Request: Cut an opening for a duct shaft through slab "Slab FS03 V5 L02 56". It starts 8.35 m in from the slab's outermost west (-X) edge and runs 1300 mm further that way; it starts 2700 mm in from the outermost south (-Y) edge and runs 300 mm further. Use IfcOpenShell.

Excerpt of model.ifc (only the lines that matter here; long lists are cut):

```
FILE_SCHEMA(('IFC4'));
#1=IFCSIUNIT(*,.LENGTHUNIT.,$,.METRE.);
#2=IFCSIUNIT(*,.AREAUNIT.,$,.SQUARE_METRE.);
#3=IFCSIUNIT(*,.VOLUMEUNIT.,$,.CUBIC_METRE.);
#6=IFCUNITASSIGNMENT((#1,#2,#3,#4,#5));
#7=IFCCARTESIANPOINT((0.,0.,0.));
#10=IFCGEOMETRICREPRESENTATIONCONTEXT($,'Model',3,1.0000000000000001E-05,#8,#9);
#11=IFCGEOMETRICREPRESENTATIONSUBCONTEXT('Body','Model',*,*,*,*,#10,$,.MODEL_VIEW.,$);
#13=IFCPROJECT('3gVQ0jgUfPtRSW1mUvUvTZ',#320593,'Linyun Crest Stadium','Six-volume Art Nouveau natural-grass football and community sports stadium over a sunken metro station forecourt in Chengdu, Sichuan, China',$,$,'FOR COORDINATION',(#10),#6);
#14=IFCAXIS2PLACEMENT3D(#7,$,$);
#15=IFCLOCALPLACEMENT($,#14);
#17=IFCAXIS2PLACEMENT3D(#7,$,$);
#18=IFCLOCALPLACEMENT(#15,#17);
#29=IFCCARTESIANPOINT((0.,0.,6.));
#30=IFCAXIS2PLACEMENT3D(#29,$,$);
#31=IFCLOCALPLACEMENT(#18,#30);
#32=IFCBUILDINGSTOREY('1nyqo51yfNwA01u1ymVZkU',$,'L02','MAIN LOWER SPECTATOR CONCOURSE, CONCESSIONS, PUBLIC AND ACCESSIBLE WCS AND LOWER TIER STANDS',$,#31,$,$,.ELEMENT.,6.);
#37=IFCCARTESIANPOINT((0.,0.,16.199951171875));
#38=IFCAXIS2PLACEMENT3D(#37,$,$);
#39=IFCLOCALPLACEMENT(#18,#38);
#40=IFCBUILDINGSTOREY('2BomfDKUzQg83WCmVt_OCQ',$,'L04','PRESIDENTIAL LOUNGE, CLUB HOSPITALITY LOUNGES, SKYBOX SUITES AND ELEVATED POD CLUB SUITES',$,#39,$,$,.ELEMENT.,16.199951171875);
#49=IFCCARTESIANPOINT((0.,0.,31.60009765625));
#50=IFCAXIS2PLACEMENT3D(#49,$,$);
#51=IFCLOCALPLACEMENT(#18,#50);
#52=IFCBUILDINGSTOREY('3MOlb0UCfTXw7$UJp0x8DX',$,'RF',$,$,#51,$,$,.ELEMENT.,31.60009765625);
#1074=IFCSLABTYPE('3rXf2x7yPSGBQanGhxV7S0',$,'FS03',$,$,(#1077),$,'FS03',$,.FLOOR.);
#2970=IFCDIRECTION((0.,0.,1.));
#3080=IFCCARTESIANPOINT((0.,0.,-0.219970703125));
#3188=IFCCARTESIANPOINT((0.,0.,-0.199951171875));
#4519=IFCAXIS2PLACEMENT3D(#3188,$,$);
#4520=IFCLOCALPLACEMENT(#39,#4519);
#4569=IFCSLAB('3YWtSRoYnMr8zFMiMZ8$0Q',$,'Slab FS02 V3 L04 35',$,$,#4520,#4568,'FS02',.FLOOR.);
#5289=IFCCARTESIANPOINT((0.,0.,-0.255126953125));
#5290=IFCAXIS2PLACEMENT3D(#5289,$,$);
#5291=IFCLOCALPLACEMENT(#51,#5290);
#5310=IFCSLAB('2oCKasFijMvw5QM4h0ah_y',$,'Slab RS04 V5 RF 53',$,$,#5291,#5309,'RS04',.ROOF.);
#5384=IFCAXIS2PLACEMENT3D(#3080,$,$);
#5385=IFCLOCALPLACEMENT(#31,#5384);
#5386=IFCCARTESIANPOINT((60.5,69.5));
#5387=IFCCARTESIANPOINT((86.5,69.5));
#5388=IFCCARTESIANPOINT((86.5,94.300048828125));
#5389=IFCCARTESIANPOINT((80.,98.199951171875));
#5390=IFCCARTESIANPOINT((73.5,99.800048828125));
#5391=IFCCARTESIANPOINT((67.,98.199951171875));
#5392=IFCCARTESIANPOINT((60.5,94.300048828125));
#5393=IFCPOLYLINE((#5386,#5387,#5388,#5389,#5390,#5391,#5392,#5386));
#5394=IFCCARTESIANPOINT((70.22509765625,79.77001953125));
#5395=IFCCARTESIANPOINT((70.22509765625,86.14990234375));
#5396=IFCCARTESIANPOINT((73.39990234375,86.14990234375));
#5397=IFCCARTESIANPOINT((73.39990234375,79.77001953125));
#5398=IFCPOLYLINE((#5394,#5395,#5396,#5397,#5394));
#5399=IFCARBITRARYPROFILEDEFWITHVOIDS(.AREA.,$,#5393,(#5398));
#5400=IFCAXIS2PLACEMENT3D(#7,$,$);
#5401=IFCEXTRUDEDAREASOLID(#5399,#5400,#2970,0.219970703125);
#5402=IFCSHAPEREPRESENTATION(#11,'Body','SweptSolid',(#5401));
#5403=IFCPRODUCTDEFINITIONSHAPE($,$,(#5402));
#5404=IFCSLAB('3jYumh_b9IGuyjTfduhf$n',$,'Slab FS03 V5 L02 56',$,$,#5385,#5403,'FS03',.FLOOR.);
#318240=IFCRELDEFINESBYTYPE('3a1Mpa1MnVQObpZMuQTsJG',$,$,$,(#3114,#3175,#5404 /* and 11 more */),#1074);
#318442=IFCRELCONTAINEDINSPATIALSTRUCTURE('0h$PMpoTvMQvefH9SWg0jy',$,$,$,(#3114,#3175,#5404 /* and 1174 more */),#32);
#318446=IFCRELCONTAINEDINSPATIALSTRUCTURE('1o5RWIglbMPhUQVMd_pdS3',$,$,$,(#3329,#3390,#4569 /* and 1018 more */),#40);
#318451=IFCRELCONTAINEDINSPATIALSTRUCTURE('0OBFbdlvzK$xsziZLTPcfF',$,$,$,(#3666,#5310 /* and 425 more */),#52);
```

```python
import numpy as np
import ifcopenshell
import ifcopenshell.api.feature
import ifcopenshell.api.geometry
import ifcopenshell.api.root
import ifcopenshell.geom
import ifcopenshell.util.placement
import ifcopenshell.util.representation
import ifcopenshell.util.shape
import ifcopenshell.util.unit

model = ifcopenshell.open("model.ifc")
unit_scale = ifcopenshell.util.unit.calculate_unit_scale(model)
settings = ifcopenshell.geom.settings()


def volume(element):
    """Net volume in cubic metres, openings subtracted."""
    shape = ifcopenshell.geom.create_shape(settings, element)
    return ifcopenshell.util.shape.get_volume(shape.geometry)


slab = model.by_id(5404)
before = volume(slab)

# Extent in the slab's own axes, in metres. The edges named are its -X and -Y sides.
slab_shape = ifcopenshell.geom.create_shape(settings, slab)
vertices = ifcopenshell.util.shape.get_vertices(slab_shape.geometry)
x_min, y_min, bottom = vertices.min(axis=0)
top = vertices[:, 2].max()

opening = ifcopenshell.api.root.create_entity(model, ifc_class="IfcOpeningElement", name="Duct shaft opening", predefined_type="OPENING")
context = ifcopenshell.util.representation.get_context(model, "Model", "Body", "MODEL_VIEW")
width, depth = 1.3, 0.3
outline = [(0.0, 0.0), (width, 0.0), (width, depth), (0.0, depth), (0.0, 0.0)]
# Overshoot both faces by 50 mm so the cut is clean.
shape = ifcopenshell.api.geometry.add_slab_representation(
    model, context=context, depth=top - bottom + 0.1, polyline=outline
)
ifcopenshell.api.geometry.assign_representation(model, product=opening, representation=shape)

matrix = ifcopenshell.util.placement.get_local_placement(slab.ObjectPlacement)
matrix[:, 3] = matrix @ np.append(np.array([x_min + 8.35, y_min + 2.7, bottom - 0.05]) / unit_scale, 1.0)
ifcopenshell.api.geometry.edit_object_placement(model, product=opening, matrix=matrix, is_si=False)
ifcopenshell.api.feature.add_feature(model, feature=opening, element=slab)

after = volume(slab)

print(f"slab volume {before:.3f} -> {after:.3f} m3")

model.write("model-out.ifc")
```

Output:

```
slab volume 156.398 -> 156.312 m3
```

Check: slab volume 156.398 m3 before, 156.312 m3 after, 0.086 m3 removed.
